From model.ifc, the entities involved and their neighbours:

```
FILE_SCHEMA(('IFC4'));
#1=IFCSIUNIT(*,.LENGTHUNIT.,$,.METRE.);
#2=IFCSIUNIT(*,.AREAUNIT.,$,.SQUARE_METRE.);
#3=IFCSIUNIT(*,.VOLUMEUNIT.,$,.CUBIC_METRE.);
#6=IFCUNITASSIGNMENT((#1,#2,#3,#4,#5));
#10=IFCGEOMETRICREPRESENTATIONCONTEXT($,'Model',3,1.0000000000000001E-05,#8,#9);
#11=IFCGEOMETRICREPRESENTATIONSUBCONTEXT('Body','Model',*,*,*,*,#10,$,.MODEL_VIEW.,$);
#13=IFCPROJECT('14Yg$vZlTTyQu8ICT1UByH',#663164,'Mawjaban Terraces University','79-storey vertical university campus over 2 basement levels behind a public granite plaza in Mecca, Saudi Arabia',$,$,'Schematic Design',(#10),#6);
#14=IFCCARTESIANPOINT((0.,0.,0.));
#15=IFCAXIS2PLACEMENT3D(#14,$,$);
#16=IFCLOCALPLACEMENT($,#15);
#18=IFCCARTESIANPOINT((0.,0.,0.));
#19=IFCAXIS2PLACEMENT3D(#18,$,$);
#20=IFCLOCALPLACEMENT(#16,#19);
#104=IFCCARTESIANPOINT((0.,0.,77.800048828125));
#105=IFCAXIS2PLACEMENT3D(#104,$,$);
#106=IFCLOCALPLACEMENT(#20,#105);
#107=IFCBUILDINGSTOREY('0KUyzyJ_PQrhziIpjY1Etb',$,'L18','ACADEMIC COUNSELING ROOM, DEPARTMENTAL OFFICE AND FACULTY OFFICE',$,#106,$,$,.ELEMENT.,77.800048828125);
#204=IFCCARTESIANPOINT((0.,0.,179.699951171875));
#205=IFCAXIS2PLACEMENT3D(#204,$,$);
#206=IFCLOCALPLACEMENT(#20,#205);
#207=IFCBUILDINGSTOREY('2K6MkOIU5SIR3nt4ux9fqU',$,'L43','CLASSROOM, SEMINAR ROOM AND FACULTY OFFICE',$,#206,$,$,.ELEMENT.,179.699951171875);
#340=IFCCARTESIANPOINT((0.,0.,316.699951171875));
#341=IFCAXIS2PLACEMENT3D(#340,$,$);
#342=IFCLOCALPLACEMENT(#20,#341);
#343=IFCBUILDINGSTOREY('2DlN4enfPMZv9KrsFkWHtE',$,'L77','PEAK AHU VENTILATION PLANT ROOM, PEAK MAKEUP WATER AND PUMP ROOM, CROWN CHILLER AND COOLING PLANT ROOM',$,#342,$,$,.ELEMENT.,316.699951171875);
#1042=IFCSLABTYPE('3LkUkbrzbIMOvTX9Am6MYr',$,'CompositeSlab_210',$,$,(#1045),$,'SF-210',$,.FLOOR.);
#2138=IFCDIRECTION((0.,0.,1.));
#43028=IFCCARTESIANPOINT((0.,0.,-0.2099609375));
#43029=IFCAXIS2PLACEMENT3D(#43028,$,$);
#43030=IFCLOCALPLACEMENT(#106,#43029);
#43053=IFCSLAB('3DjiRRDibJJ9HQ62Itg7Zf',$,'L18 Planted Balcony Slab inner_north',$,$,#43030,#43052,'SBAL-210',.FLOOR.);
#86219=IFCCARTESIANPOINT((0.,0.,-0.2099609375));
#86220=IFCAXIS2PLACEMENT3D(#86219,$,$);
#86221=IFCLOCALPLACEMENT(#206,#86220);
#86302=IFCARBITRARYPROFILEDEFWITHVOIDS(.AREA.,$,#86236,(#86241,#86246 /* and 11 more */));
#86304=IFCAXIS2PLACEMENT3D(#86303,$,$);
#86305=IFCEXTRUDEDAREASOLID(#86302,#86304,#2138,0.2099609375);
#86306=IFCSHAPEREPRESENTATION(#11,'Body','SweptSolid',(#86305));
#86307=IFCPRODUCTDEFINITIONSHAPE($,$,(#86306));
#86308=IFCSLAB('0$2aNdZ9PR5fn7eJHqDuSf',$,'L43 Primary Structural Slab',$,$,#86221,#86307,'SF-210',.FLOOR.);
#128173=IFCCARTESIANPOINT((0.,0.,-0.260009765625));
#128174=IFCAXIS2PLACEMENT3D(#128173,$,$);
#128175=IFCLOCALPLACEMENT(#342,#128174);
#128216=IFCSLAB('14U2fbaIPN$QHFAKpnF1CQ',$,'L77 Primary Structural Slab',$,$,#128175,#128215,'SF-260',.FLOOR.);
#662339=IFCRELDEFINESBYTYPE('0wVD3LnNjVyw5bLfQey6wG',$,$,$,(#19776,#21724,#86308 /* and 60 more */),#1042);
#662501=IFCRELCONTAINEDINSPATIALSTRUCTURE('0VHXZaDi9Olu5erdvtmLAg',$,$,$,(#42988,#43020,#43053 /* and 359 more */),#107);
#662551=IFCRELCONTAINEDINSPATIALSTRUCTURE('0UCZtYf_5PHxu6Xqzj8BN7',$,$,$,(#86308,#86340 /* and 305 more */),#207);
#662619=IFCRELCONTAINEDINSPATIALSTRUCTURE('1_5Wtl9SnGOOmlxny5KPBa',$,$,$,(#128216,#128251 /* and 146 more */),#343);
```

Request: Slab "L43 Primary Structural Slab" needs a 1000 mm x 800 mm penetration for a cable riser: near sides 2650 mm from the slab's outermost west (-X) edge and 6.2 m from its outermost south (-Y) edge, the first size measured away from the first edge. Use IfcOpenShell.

```python
import numpy as np
import ifcopenshell
import ifcopenshell.api.feature
import ifcopenshell.api.geometry
import ifcopenshell.api.root
import ifcopenshell.geom
import ifcopenshell.util.placement
import ifcopenshell.util.representation
import ifcopenshell.util.shape
import ifcopenshell.util.unit

model = ifcopenshell.open("model.ifc")
unit_scale = ifcopenshell.util.unit.calculate_unit_scale(model)
settings = ifcopenshell.geom.settings()


def volume(element):
    """Net volume in cubic metres, openings subtracted."""
    shape = ifcopenshell.geom.create_shape(settings, element)
    return ifcopenshell.util.shape.get_volume(shape.geometry)


slab = model.by_guid("0$2aNdZ9PR5fn7eJHqDuSf")
before = volume(slab)

# Extent in the slab's own axes, in metres. The edges named are its -X and -Y sides.
slab_shape = ifcopenshell.geom.create_shape(settings, slab)
vertices = ifcopenshell.util.shape.get_vertices(slab_shape.geometry)
x_min, y_min, bottom = vertices.min(axis=0)
top = vertices[:, 2].max()

opening = ifcopenshell.api.root.create_entity(model, ifc_class="IfcOpeningElement", name="Cable riser opening", predefined_type="OPENING")
context = ifcopenshell.util.representation.get_context(model, "Model", "Body", "MODEL_VIEW")
width, depth = 1, 0.8
outline = [(0.0, 0.0), (width, 0.0), (width, depth), (0.0, depth), (0.0, 0.0)]
# Overshoot both faces by 50 mm so the cut is clean.
shape = ifcopenshell.api.geometry.add_slab_representation(
    model, context=context, depth=top - bottom + 0.1, polyline=outline
)
ifcopenshell.api.geometry.assign_representation(model, product=opening, representation=shape)

matrix = ifcopenshell.util.placement.get_local_placement(slab.ObjectPlacement)
matrix[:, 3] = matrix @ np.append(np.array([x_min + 2.65, y_min + 6.2, bottom - 0.05]) / unit_scale, 1.0)
ifcopenshell.api.geometry.edit_object_placement(model, product=opening, matrix=matrix, is_si=False)
ifcopenshell.api.feature.add_feature(model, feature=opening, element=slab)

after = volume(slab)

print(f"slab volume {before:.3f} -> {after:.3f} m3")

model.write("model-out.ifc")
```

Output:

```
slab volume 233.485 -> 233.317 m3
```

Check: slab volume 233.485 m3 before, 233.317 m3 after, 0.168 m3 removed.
